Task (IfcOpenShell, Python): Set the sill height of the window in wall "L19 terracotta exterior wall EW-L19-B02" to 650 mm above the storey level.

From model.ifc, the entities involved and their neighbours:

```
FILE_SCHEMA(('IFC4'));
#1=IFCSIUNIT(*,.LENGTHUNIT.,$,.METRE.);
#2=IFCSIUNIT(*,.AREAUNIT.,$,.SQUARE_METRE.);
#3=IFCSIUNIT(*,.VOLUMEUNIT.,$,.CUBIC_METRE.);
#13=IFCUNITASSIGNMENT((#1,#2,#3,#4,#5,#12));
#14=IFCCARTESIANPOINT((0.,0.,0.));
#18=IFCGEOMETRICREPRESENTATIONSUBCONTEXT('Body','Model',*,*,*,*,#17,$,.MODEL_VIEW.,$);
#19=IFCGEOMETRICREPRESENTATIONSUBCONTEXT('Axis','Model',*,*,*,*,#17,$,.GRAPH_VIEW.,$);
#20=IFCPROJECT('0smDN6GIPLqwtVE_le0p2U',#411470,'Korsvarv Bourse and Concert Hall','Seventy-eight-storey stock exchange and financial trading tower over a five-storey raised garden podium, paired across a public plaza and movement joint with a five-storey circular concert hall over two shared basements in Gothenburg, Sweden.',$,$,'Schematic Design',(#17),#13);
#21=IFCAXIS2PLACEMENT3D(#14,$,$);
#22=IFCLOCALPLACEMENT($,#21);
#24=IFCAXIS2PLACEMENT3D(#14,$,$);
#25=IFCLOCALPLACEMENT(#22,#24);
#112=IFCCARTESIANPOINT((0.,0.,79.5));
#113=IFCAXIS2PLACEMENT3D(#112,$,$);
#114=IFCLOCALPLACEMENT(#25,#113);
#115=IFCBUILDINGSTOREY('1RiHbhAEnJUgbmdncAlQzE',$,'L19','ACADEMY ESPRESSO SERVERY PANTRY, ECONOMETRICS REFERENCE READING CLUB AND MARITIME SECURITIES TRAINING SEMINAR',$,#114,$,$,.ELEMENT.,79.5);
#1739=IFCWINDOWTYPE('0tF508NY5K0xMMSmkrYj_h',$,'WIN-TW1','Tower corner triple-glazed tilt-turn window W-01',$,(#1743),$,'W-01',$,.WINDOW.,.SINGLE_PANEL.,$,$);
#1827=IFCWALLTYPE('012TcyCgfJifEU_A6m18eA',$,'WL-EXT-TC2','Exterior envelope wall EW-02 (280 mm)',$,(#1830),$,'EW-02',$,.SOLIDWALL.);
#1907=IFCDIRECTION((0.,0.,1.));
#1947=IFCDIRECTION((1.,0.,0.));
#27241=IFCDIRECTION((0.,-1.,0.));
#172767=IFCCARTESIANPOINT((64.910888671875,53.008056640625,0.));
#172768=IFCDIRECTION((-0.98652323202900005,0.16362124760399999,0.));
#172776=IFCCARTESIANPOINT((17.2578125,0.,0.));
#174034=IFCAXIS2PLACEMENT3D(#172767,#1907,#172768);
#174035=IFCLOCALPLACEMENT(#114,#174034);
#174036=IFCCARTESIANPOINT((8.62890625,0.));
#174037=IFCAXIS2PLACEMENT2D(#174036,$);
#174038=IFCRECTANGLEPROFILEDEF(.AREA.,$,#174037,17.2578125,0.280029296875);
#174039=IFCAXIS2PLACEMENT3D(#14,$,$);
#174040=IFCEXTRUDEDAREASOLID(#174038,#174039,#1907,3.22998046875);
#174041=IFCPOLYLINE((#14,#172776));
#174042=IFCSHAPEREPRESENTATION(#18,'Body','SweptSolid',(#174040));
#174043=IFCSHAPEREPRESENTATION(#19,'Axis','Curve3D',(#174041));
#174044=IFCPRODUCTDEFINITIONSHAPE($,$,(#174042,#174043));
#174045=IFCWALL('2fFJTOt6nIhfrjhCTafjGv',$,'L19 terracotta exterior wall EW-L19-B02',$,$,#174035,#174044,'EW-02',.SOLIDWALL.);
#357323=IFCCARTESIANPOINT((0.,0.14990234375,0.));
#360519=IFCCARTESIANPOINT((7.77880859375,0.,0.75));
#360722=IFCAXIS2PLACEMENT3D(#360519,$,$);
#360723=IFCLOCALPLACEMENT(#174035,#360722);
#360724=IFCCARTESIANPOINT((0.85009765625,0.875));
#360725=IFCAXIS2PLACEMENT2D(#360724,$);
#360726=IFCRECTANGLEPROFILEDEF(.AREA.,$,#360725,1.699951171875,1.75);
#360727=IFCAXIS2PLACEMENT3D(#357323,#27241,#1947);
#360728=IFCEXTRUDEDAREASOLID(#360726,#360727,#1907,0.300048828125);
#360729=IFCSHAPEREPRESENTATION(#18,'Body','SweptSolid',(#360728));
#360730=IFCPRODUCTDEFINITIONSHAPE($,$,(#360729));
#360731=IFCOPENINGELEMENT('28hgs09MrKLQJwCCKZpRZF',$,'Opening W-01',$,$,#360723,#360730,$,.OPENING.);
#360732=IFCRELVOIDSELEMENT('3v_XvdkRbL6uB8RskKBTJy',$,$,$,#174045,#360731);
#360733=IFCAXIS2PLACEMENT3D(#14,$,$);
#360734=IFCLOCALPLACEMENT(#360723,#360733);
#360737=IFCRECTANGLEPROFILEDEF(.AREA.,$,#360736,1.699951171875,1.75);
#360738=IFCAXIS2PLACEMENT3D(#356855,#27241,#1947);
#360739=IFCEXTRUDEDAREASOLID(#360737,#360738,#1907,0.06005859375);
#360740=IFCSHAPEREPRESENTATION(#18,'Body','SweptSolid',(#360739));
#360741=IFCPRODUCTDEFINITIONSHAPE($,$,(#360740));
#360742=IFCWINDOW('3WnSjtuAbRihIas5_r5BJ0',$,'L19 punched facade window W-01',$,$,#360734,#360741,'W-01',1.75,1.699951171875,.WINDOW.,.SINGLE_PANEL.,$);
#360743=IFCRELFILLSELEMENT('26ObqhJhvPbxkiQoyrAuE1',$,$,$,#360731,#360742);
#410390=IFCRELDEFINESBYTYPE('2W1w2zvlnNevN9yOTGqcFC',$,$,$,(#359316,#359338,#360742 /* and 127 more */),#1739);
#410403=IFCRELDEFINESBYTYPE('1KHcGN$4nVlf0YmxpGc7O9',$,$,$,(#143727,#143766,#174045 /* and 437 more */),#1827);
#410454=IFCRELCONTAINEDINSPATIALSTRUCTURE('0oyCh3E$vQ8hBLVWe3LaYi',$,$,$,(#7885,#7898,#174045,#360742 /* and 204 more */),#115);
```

```python
import numpy as np
import ifcopenshell
import ifcopenshell.api.geometry
import ifcopenshell.geom
import ifcopenshell.util.element
import ifcopenshell.util.placement
import ifcopenshell.util.shape
import ifcopenshell.util.unit

model = ifcopenshell.open("model.ifc")
unit_scale = ifcopenshell.util.unit.calculate_unit_scale(model)

window = model.by_guid("3WnSjtuAbRihIas5_r5BJ0")
opening = window.FillsVoids[0].RelatingOpeningElement
storey = ifcopenshell.util.element.get_container(window, ifc_class="IfcBuildingStorey")
level = ifcopenshell.util.placement.get_local_placement(storey.ObjectPlacement)[2, 3]

# The opening's origin need not be at the sill, so measure its lowest point.
shape = ifcopenshell.geom.create_shape(ifcopenshell.geom.settings(), opening)
bottom = ifcopenshell.util.shape.get_shape_bottom_elevation(shape, shape.geometry) / unit_scale
dz = level + 0.65 - bottom

shift = np.array([0.0, 0.0, dz])
# The window is placed relative to its opening, so it follows when the opening moves.
matrix = ifcopenshell.util.placement.get_local_placement(opening.ObjectPlacement)
matrix[:3, 3] += shift
ifcopenshell.api.geometry.edit_object_placement(
    model, product=opening, matrix=matrix, is_si=False, should_transform_children=True
)

print(f"moved by {dz * unit_scale:+.3f} m")

model.write("model_updated.ifc")
```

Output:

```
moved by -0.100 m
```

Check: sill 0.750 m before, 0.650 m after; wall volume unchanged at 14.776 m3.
